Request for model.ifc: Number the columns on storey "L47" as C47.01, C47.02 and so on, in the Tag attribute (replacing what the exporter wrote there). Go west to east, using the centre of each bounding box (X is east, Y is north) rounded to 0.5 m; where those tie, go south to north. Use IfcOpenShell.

First a look at what the model holds.

```python
import ifcopenshell
import ifcopenshell.util.element
import ifcopenshell.util.placement

model = ifcopenshell.open("model.ifc")
print(model.schema)
storey = next(s for s in model.by_type("IfcBuildingStorey") if s.Name == "L47")
columns = [e for e in ifcopenshell.util.element.get_decomposition(storey) if e.is_a("IfcColumn")]
for e in sorted(columns, key=lambda e: e.id()):
    origin = ifcopenshell.util.placement.get_local_placement(e.ObjectPlacement)[:3, 3]
    print(e.id(), e.Tag, e.Name, origin.round(2) + 0.0, sep=" | ")
```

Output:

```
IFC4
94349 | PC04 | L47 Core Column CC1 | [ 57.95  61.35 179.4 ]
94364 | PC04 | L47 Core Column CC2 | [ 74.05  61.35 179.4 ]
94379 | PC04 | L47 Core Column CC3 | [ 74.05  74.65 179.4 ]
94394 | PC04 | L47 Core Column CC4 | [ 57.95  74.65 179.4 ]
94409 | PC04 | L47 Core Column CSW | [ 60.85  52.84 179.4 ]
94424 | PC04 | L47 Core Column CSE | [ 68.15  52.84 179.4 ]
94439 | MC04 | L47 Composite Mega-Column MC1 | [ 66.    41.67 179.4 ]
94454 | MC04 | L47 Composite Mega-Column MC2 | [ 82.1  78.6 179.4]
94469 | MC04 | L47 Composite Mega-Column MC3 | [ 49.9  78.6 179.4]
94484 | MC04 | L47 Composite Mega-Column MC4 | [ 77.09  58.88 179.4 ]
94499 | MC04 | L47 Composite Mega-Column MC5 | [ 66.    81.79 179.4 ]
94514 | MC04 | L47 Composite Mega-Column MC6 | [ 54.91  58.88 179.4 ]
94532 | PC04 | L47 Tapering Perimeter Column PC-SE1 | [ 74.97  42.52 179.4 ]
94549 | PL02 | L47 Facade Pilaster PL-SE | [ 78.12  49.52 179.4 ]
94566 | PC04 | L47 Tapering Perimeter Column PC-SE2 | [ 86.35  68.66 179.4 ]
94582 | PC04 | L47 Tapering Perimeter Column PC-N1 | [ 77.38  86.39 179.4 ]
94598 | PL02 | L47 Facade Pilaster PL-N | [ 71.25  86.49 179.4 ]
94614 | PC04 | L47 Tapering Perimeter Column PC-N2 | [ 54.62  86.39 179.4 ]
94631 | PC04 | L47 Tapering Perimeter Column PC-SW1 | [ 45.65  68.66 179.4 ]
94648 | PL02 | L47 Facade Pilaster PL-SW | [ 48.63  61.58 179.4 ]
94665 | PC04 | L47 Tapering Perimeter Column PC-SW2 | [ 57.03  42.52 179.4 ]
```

```python
import ifcopenshell
import ifcopenshell.geom
import ifcopenshell.util.element
import ifcopenshell.util.shape

model = ifcopenshell.open("model.ifc")
settings = ifcopenshell.geom.settings()
settings.set("use-world-coords", True)


def centre(element):
    shape = ifcopenshell.geom.create_shape(settings, element)
    return ifcopenshell.util.shape.get_bbox_centroid(shape.geometry)


storey = next(s for s in model.by_type("IfcBuildingStorey") if s.Name == "L47")
columns = [e for e in ifcopenshell.util.element.get_decomposition(storey) if e.is_a("IfcColumn")]

# Insertion points can sit at a corner or the storey origin, so sort by the geometry (in metres).
centres = {e: centre(e) for e in columns}
columns.sort(key=lambda e: (round(centres[e][0] / 0.5), centres[e][1]))

for i, e in enumerate(columns, start=1):
    number = f"C47.{i:02d}"
    e.Tag = number
    print(e.id(), number)

model.write("model_v2.ifc")
```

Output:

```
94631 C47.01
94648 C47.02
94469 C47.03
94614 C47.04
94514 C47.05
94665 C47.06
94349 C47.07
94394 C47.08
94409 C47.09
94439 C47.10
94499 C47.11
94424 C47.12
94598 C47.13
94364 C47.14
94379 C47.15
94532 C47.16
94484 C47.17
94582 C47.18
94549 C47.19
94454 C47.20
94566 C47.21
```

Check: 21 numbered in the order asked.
